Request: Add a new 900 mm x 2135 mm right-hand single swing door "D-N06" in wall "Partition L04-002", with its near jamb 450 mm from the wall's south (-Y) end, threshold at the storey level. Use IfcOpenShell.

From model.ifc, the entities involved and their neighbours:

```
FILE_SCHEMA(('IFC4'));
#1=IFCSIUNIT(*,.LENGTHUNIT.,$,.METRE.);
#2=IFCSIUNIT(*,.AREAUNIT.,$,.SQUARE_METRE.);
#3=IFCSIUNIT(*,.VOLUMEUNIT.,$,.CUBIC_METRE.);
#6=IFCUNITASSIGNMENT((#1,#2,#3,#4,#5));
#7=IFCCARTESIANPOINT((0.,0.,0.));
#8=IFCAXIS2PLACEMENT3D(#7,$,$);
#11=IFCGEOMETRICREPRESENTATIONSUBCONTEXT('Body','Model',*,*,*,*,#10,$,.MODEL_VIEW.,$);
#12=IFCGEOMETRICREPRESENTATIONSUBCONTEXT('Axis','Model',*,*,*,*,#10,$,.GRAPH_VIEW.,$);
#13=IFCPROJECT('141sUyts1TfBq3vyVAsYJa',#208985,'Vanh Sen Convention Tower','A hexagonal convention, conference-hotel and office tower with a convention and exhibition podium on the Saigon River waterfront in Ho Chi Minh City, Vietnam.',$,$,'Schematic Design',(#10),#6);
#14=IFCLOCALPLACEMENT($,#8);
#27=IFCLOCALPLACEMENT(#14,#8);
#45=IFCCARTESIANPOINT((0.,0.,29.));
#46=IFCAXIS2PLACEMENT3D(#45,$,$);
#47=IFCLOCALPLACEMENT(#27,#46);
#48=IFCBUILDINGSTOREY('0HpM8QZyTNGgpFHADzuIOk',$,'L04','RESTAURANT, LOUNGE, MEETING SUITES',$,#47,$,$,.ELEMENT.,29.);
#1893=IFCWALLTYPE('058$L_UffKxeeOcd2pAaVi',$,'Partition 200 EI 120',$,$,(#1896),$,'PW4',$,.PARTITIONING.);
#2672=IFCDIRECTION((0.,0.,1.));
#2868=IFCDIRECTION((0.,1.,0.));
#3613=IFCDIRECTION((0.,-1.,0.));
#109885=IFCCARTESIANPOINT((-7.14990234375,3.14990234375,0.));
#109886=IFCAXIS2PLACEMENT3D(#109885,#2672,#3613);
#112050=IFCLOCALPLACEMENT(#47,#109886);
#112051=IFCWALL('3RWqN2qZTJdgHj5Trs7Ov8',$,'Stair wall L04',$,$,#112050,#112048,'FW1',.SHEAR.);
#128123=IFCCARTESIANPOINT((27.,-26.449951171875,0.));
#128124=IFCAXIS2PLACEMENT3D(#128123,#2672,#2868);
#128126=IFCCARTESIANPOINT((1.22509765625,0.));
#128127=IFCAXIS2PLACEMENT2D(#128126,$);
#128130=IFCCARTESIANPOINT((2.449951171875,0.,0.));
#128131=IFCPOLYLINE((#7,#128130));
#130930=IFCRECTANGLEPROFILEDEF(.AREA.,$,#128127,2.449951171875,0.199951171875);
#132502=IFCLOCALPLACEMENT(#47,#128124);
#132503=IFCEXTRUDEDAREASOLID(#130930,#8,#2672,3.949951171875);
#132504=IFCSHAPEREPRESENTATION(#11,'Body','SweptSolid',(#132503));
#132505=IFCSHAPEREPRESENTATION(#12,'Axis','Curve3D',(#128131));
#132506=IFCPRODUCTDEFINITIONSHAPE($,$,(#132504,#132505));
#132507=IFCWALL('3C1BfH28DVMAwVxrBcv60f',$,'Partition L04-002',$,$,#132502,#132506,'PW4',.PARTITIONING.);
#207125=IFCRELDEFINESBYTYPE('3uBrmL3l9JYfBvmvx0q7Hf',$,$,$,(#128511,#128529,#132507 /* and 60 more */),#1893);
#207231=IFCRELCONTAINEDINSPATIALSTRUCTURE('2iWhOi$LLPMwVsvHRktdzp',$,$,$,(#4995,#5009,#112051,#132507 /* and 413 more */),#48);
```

```python
import numpy as np
import ifcopenshell
import ifcopenshell.api.feature
import ifcopenshell.api.geometry
import ifcopenshell.api.root
import ifcopenshell.api.spatial
import ifcopenshell.geom
import ifcopenshell.util.element
import ifcopenshell.util.placement
import ifcopenshell.util.representation
import ifcopenshell.util.shape
import ifcopenshell.util.unit

model = ifcopenshell.open("model.ifc")
unit_scale = ifcopenshell.util.unit.calculate_unit_scale(model)
settings = ifcopenshell.geom.settings()


def volume(element):
    """Net volume in cubic metres, openings subtracted."""
    shape = ifcopenshell.geom.create_shape(settings, element)
    return ifcopenshell.util.shape.get_volume(shape.geometry)


wall = model.by_guid("3C1BfH28DVMAwVxrBcv60f")
storey = ifcopenshell.util.element.get_container(wall, ifc_class="IfcBuildingStorey")
context = ifcopenshell.util.representation.get_context(model, "Model", "Body", "MODEL_VIEW")
before = volume(wall)

width, height, from_end, sill = 0.9, 2.135, 0.45, 0.0  # metres

# The wall runs along its own X axis, and the end named is its -X end.
wall_shape = ifcopenshell.geom.create_shape(settings, wall)
x, y, z = ifcopenshell.util.shape.get_vertices(wall_shape.geometry).T
start = x.min() + from_end
face, thickness = float(y.min()), float(y.max() - y.min())
wall_matrix = ifcopenshell.util.placement.get_local_placement(wall.ObjectPlacement)
level = ifcopenshell.util.placement.get_local_placement(storey.ObjectPlacement)[2, 3]


def in_wall(x, y):
    """Placement at x, y metres in the wall's axes, at sill height."""
    matrix = wall_matrix.copy()
    matrix[:, 3] = wall_matrix @ np.array([x / unit_scale, y / unit_scale, 0.0, 1.0])
    matrix[2, 3] = level + sill / unit_scale
    return matrix


# Opening: a box that overshoots both wall faces by 50 mm.
opening = ifcopenshell.api.root.create_entity(model, ifc_class="IfcOpeningElement", predefined_type="OPENING")
box = ifcopenshell.api.geometry.add_wall_representation(
    model, context=context, length=width, height=height, thickness=thickness + 0.1
)
ifcopenshell.api.geometry.assign_representation(model, product=opening, representation=box)
ifcopenshell.api.geometry.edit_object_placement(model, product=opening, matrix=in_wall(start, face - 0.05), is_si=False)
ifcopenshell.api.feature.add_feature(model, feature=opening, element=wall)

door = ifcopenshell.api.root.create_entity(model, ifc_class="IfcDoor", name="D-N06", predefined_type="DOOR")
door.OverallWidth, door.OverallHeight = width / unit_scale, height / unit_scale
door.OperationType = "SINGLE_SWING_RIGHT"
body = ifcopenshell.api.geometry.add_door_representation(
    model,
    context=context,
    overall_width=door.OverallWidth,
    overall_height=door.OverallHeight,
    operation_type="SINGLE_SWING_RIGHT",
    lining_properties={"LiningDepth": thickness / unit_scale, "ThresholdDepth": thickness / unit_scale},
)
ifcopenshell.api.geometry.assign_representation(model, product=door, representation=body)
ifcopenshell.api.spatial.assign_container(model, products=[door], relating_structure=storey)
ifcopenshell.api.feature.add_filling(model, opening=opening, element=door)

# The lining spans the wall, so the door starts at the wall face.
ifcopenshell.api.geometry.edit_object_placement(model, product=door, matrix=in_wall(start, face), is_si=False)

after = volume(wall)

print(f"wall volume {before:.3f} -> {after:.3f} m3")

model.write("model_rev.ifc")
```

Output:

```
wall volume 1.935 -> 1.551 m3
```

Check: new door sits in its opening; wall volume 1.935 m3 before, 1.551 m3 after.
